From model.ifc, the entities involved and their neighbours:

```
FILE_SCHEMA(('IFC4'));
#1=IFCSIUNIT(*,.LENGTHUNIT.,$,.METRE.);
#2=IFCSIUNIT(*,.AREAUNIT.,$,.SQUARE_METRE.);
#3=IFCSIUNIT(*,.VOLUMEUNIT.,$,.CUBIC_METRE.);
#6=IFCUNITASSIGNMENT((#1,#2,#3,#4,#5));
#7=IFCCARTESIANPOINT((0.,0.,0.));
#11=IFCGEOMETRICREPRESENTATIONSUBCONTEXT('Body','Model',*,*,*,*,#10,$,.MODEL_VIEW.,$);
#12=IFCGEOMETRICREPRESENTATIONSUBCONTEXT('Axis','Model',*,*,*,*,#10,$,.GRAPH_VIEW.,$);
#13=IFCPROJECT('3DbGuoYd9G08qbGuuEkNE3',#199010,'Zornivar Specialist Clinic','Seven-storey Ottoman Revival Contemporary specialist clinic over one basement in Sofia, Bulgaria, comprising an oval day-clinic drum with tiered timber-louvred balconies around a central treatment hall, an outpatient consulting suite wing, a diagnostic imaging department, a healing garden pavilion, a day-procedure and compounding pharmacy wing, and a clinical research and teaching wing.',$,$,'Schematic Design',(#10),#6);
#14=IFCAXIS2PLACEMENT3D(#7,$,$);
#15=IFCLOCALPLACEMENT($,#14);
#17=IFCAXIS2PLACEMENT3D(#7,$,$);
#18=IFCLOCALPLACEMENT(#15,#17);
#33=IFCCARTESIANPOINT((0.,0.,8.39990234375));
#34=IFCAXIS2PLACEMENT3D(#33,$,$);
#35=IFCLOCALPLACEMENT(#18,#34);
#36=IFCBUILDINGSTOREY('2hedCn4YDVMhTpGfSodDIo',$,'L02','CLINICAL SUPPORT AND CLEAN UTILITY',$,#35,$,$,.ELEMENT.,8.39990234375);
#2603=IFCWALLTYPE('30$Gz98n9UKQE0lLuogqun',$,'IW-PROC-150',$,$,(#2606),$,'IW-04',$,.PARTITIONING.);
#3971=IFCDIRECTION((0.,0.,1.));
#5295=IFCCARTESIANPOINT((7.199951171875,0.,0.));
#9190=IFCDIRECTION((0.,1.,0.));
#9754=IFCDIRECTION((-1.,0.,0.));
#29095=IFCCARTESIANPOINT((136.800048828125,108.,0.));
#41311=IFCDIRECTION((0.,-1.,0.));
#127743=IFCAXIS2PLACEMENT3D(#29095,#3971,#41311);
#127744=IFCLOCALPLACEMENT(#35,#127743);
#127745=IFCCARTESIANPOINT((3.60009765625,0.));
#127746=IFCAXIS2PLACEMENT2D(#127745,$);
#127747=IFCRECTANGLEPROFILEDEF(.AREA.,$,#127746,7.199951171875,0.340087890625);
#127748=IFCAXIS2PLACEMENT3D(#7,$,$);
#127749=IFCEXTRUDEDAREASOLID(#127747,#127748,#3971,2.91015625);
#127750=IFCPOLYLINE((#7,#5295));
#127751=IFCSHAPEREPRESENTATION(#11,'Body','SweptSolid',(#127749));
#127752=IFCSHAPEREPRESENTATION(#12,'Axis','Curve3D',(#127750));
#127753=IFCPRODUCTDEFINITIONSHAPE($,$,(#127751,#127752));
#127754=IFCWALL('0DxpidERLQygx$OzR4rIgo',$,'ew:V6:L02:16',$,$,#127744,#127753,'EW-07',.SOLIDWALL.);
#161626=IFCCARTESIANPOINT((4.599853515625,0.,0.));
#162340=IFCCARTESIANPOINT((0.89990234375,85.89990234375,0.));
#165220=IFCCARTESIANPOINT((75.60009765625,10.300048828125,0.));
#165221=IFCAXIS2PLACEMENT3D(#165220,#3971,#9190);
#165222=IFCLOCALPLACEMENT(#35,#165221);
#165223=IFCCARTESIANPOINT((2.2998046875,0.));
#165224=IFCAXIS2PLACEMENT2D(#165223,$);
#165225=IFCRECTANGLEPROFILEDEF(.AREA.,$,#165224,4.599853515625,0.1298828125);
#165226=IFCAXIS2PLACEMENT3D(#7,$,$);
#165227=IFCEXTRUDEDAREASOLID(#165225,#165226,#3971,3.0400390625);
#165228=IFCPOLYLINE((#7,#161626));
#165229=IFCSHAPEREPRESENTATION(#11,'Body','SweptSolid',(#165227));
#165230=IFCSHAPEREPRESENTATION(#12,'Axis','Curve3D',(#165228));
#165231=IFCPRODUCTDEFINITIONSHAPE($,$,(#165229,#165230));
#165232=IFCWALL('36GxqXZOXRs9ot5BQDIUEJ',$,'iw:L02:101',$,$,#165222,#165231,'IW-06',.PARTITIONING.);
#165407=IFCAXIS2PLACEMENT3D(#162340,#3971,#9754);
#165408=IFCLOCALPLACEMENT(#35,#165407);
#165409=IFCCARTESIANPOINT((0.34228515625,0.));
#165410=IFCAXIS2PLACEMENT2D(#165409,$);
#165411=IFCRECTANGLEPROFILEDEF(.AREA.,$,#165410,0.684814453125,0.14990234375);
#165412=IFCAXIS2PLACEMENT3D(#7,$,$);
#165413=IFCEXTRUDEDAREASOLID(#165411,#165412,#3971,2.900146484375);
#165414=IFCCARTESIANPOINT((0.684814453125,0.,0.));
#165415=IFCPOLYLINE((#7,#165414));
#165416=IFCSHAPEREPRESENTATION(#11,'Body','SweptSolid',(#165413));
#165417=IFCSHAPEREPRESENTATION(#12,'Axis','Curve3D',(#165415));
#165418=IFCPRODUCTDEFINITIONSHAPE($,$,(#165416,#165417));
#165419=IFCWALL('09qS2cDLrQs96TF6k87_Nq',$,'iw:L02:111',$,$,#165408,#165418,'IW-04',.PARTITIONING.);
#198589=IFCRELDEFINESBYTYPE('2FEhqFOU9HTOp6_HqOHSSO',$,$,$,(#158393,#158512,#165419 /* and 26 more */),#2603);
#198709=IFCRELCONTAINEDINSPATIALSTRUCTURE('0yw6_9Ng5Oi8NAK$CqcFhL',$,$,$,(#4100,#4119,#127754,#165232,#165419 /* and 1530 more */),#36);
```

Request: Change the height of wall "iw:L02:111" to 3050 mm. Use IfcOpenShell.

```python
import ifcopenshell
import ifcopenshell.geom
import ifcopenshell.util.representation
import ifcopenshell.util.shape

model = ifcopenshell.open("model.ifc")
settings = ifcopenshell.geom.settings()


def volume(element):
    """Net volume in cubic metres, openings subtracted."""
    shape = ifcopenshell.geom.create_shape(settings, element)
    return ifcopenshell.util.shape.get_volume(shape.geometry)


wall = model.by_guid("09qS2cDLrQs96TF6k87_Nq")
before = volume(wall)

body = ifcopenshell.util.representation.get_representation(wall, "Model", "Body")
solid = body.Items[0]
old_height = solid.Depth
solid.Depth = 3.05
after = volume(wall)

print(f"height {old_height:g} -> {solid.Depth:g}, volume {before:.3f} -> {after:.3f} m3")

model.write("model_updated.ifc")
```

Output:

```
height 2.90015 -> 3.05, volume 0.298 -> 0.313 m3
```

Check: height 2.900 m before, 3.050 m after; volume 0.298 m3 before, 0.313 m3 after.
